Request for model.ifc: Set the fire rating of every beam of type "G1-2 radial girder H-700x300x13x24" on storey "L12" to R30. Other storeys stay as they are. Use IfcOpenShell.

First a look at what the model holds.

```python
import ifcopenshell
import ifcopenshell.util.element

model = ifcopenshell.open("model.ifc")
print(model.schema)
storey = next(s for s in model.by_type("IfcBuildingStorey") if s.Name == "L12")
beams = [e for e in ifcopenshell.util.element.get_decomposition(storey) if e.is_a("IfcBeam")]
seen = {}
for e in beams:
    element_type = ifcopenshell.util.element.get_type(e)
    key = (element_type.Name if element_type != e and element_type else None, ifcopenshell.util.element.get_pset(e, "Pset_BeamCommon", "FireRating"))
    seen[key] = seen.get(key, 0) + 1
for (name, value), count in sorted(seen.items(), key=str):
    print(count, "x", name, "|", value)
```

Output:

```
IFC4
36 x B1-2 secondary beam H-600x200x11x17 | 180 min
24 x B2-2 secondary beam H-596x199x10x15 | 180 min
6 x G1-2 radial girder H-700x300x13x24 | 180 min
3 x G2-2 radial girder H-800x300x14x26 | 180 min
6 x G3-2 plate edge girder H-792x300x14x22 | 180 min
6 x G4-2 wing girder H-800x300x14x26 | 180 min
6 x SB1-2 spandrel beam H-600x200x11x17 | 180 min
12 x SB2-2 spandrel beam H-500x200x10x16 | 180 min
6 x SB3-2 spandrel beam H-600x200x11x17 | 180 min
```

```python
import ifcopenshell
import ifcopenshell.api.pset
import ifcopenshell.util.element

model = ifcopenshell.open("model.ifc")

storey = next(s for s in model.by_type("IfcBuildingStorey") if s.Name == "L12")
beams = [e for e in ifcopenshell.util.element.get_decomposition(storey) if e.is_a("IfcBeam")]

count = 0
for e in beams:
    element_type = ifcopenshell.util.element.get_type(e)
    if element_type in (None, e) or element_type.Name != "G1-2 radial girder H-700x300x13x24":
        continue
    found = ifcopenshell.util.element.get_pset(e, "Pset_BeamCommon", should_inherit=False)
    if found:
        pset = model.by_id(found["id"])
        if len(ifcopenshell.util.element.get_elements_by_pset(pset)) > 1:
            pset = ifcopenshell.api.pset.unshare_pset(model, products=[e], pset=pset)[0]
    else:
        pset = ifcopenshell.api.pset.add_pset(model, product=e, name="Pset_BeamCommon")
    ifcopenshell.api.pset.edit_pset(model, pset=pset, properties={"FireRating": "R30"})
    count += 1

print(count, "beams updated")

model.write("model_rev.ifc")
```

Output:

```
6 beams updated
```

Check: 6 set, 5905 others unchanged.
